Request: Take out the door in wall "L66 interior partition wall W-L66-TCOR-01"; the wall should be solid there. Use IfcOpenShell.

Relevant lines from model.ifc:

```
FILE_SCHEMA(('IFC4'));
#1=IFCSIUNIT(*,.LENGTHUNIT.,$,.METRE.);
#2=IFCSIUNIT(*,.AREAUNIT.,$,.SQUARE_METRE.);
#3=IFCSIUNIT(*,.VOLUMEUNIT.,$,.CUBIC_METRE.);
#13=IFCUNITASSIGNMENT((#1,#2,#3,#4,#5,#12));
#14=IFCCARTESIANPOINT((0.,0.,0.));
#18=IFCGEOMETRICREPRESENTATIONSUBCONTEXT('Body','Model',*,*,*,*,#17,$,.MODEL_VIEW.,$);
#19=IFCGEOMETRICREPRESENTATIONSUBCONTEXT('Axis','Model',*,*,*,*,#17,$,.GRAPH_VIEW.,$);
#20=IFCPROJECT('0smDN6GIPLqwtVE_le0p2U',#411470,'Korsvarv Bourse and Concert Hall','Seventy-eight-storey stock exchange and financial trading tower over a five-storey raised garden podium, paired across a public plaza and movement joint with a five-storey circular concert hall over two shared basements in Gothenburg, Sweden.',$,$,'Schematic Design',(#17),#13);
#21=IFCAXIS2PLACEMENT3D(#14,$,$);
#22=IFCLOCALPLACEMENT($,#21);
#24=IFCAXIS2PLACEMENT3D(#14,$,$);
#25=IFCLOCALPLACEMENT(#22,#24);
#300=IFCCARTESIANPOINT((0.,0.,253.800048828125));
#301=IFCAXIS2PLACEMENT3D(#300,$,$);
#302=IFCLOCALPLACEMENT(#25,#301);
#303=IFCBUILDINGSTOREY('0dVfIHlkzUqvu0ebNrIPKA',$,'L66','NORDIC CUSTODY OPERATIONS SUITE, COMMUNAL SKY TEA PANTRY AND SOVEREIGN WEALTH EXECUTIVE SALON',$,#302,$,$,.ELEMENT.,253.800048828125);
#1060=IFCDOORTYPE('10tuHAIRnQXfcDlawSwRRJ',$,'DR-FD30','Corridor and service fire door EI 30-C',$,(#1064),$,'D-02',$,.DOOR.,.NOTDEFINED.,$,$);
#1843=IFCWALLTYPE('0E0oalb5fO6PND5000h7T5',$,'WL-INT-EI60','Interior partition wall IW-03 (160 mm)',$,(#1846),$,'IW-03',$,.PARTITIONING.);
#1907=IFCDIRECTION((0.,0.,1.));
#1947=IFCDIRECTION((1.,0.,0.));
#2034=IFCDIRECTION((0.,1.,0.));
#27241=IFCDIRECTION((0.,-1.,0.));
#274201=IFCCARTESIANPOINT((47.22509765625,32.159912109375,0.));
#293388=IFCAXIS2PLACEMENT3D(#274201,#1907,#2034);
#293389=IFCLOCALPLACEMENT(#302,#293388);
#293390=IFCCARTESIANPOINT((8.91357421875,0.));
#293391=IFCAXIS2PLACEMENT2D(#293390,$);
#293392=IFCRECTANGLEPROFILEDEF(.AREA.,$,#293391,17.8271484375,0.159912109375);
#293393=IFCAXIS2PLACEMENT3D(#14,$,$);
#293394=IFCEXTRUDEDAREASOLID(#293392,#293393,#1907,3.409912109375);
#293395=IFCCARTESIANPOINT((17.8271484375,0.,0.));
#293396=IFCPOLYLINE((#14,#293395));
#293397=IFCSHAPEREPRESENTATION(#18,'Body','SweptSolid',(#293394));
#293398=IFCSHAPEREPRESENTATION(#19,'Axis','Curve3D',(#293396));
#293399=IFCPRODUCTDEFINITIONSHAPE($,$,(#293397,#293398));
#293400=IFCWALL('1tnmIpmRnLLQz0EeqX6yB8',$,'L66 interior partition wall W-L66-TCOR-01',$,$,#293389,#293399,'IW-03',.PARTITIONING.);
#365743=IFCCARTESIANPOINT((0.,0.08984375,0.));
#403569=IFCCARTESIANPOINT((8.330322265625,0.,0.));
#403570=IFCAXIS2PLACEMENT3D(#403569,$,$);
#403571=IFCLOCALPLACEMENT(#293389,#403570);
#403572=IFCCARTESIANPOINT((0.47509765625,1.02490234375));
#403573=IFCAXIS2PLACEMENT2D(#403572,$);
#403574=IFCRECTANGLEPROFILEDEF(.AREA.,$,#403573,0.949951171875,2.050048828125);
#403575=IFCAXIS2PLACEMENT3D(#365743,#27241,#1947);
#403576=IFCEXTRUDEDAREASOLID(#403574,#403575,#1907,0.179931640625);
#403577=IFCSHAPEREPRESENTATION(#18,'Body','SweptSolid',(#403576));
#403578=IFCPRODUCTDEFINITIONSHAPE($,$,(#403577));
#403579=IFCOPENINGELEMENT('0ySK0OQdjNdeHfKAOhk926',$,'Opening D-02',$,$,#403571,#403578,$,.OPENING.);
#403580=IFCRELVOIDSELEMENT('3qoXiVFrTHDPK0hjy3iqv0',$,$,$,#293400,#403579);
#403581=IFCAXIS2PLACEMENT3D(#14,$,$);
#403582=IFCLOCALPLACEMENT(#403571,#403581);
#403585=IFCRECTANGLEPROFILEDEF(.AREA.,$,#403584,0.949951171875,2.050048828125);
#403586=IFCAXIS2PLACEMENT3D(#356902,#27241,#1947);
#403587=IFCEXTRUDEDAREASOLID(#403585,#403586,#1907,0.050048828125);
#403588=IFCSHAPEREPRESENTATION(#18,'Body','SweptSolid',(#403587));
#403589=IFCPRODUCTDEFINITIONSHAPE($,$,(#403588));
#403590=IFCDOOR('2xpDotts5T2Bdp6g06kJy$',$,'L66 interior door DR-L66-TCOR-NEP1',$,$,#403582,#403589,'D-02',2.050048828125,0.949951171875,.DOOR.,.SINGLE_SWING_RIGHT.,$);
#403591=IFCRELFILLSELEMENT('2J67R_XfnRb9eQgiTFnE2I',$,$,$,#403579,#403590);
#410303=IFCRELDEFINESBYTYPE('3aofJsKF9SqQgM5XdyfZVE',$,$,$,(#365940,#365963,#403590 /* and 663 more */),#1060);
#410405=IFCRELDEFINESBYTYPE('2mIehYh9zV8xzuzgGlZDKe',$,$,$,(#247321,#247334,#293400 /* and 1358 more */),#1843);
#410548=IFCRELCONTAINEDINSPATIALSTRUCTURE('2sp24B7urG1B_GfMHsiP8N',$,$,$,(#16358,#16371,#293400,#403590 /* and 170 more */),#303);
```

```python
import ifcopenshell
import ifcopenshell.api.feature
import ifcopenshell.api.root
import ifcopenshell.geom
import ifcopenshell.util.shape

model = ifcopenshell.open("model.ifc")
settings = ifcopenshell.geom.settings()


def volume(element):
    """Net volume in cubic metres, openings subtracted."""
    shape = ifcopenshell.geom.create_shape(settings, element)
    return ifcopenshell.util.shape.get_volume(shape.geometry)


door = model.by_id(403590)
opening = door.FillsVoids[0].RelatingOpeningElement
wall = opening.VoidsElements[0].RelatingBuildingElement
before = volume(wall)

ifcopenshell.api.root.remove_product(model, product=door)
ifcopenshell.api.feature.remove_feature(model, feature=opening)

after = volume(wall)

print(f"wall volume {before:.3f} -> {after:.3f} m3")

model.write("model_updated.ifc")
```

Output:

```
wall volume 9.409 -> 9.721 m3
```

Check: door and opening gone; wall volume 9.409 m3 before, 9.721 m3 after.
